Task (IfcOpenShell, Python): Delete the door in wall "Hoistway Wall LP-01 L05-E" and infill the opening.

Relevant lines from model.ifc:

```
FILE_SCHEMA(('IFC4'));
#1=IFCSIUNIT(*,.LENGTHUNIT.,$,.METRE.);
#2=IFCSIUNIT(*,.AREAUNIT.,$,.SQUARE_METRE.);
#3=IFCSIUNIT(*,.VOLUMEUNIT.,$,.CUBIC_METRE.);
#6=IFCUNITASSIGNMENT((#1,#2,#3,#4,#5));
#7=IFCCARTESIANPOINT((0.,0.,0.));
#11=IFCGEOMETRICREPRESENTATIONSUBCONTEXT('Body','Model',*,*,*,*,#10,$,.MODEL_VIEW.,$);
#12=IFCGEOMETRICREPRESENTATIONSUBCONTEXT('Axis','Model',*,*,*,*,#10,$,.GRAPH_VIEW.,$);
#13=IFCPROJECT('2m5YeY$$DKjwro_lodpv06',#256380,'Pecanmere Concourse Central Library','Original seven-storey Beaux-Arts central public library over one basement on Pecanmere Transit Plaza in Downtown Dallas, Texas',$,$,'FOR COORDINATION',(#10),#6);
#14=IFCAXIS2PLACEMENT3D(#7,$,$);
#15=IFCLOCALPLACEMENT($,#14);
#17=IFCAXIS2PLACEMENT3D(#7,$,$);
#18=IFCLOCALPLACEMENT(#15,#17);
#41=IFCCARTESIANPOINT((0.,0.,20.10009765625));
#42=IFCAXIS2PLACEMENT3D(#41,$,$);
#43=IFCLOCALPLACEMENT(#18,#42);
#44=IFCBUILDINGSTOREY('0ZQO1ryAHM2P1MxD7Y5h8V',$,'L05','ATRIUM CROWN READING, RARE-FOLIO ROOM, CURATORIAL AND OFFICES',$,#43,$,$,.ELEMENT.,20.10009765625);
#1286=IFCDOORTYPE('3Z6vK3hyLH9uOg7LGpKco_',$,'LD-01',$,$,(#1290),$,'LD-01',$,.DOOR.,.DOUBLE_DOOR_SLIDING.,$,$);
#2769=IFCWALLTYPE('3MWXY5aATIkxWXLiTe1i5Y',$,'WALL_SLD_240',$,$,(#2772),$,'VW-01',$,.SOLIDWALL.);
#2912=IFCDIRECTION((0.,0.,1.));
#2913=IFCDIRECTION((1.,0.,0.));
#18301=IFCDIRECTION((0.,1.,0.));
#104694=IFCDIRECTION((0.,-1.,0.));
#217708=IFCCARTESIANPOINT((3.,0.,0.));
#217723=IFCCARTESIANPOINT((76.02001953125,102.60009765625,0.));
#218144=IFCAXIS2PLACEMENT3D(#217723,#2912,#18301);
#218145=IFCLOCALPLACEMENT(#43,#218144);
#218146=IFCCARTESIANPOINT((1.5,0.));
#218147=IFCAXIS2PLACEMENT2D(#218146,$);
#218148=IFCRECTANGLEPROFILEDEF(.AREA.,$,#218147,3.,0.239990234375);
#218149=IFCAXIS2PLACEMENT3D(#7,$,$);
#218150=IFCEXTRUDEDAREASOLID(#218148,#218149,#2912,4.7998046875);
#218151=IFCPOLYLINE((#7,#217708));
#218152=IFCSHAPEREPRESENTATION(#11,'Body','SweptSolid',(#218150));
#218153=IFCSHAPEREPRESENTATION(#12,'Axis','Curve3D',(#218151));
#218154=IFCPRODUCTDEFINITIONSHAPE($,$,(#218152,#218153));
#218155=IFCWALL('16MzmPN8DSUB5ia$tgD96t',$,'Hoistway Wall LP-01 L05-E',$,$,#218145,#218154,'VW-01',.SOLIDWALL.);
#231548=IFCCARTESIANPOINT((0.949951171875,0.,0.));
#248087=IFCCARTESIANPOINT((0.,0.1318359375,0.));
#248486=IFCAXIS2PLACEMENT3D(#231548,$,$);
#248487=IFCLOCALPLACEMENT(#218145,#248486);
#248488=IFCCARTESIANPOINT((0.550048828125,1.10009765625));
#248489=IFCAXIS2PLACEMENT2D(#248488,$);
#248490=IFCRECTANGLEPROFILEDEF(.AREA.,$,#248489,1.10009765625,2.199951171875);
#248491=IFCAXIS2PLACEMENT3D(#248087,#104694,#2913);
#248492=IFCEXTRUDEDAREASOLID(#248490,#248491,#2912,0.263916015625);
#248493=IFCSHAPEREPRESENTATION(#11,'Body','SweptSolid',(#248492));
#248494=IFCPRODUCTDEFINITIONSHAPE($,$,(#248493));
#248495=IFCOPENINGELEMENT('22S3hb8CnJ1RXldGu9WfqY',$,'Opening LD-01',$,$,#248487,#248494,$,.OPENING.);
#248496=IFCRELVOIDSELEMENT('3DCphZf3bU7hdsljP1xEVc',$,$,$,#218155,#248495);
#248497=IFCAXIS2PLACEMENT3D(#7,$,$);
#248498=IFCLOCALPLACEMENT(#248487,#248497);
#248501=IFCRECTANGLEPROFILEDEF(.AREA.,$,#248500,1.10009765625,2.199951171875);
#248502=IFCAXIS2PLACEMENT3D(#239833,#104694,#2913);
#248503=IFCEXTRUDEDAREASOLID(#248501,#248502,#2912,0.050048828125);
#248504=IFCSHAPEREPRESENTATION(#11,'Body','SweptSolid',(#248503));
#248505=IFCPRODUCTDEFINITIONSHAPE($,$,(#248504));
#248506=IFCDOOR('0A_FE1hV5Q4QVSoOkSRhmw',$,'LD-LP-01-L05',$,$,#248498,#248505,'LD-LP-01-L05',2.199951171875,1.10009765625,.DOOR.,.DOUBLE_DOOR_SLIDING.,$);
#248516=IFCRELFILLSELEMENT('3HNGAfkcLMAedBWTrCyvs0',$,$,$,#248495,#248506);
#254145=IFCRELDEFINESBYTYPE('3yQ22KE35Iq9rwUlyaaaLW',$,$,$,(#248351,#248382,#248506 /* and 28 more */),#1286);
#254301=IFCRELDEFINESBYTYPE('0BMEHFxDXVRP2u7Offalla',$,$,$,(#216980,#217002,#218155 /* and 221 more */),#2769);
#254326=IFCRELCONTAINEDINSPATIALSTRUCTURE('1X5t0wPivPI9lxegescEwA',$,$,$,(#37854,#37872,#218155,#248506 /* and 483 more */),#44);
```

```python
import ifcopenshell
import ifcopenshell.api.feature
import ifcopenshell.api.root
import ifcopenshell.geom
import ifcopenshell.util.shape

model = ifcopenshell.open("model.ifc")
settings = ifcopenshell.geom.settings()


def volume(element):
    """Net volume in cubic metres, openings subtracted."""
    shape = ifcopenshell.geom.create_shape(settings, element)
    return ifcopenshell.util.shape.get_volume(shape.geometry)


door = model.by_guid("0A_FE1hV5Q4QVSoOkSRhmw")
opening = door.FillsVoids[0].RelatingOpeningElement
wall = opening.VoidsElements[0].RelatingBuildingElement
before = volume(wall)

ifcopenshell.api.root.remove_product(model, product=door)
ifcopenshell.api.feature.remove_feature(model, feature=opening)

after = volume(wall)

print(f"wall volume {before:.3f} -> {after:.3f} m3")

model.write("model_updated.ifc")
```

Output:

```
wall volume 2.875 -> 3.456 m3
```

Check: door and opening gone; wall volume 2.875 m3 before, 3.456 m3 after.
